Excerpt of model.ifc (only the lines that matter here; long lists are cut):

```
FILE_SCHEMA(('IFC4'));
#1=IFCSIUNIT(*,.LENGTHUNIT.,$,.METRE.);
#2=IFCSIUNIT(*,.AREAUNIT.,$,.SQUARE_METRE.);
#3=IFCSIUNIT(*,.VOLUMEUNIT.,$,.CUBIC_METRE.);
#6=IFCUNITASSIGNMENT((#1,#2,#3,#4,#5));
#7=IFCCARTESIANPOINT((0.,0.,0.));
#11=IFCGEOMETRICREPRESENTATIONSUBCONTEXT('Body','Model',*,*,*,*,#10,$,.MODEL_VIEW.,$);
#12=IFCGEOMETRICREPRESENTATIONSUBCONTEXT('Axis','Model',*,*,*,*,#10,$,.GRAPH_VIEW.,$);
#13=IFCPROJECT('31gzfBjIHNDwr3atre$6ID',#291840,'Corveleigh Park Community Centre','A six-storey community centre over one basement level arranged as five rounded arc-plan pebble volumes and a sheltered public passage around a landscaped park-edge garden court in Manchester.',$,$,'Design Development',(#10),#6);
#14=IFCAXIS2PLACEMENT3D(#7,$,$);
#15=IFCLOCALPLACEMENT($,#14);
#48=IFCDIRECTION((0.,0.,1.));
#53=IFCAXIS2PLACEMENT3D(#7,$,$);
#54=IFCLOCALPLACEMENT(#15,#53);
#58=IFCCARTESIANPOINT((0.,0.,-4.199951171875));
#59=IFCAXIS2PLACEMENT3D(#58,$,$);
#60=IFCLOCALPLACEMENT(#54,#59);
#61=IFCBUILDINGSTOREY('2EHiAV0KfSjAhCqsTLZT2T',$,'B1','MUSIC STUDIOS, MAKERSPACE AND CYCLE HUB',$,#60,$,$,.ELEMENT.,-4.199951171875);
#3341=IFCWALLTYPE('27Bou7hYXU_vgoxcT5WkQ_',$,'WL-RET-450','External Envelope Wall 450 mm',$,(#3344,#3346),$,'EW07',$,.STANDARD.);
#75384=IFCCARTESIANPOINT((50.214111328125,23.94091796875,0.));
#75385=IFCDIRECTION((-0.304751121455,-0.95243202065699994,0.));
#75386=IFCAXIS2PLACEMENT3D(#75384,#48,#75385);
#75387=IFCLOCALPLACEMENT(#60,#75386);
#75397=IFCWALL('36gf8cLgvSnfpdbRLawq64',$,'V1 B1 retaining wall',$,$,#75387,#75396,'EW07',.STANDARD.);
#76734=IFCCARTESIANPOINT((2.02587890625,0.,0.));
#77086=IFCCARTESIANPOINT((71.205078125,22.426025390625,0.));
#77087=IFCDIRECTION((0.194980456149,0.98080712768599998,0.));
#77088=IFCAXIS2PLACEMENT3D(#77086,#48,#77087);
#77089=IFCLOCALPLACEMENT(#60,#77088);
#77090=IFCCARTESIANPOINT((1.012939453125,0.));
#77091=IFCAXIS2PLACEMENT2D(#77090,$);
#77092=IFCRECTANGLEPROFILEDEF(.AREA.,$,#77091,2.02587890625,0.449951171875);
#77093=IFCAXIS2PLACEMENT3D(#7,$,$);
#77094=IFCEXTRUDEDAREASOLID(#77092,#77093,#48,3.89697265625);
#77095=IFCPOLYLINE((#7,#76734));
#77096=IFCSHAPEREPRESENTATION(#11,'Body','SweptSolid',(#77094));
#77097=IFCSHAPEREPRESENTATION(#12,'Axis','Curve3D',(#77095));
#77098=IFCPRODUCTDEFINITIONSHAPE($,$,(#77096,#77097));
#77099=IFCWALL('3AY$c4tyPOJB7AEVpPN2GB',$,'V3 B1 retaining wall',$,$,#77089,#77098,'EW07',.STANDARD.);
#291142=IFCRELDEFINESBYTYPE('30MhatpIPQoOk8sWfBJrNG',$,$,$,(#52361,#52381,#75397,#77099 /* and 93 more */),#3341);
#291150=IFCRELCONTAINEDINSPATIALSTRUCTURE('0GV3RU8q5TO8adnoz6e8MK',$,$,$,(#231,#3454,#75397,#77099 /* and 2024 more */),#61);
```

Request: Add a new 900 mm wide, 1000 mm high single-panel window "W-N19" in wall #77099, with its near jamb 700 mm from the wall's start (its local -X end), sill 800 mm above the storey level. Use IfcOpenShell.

```python
import numpy as np
import ifcopenshell
import ifcopenshell.api.feature
import ifcopenshell.api.geometry
import ifcopenshell.api.root
import ifcopenshell.api.spatial
import ifcopenshell.geom
import ifcopenshell.util.element
import ifcopenshell.util.placement
import ifcopenshell.util.representation
import ifcopenshell.util.shape
import ifcopenshell.util.unit

model = ifcopenshell.open("model.ifc")
unit_scale = ifcopenshell.util.unit.calculate_unit_scale(model)
settings = ifcopenshell.geom.settings()


def volume(element):
    """Net volume in cubic metres, openings subtracted."""
    shape = ifcopenshell.geom.create_shape(settings, element)
    return ifcopenshell.util.shape.get_volume(shape.geometry)


wall = model.by_guid("3AY$c4tyPOJB7AEVpPN2GB")
storey = ifcopenshell.util.element.get_container(wall, ifc_class="IfcBuildingStorey")
context = ifcopenshell.util.representation.get_context(model, "Model", "Body", "MODEL_VIEW")
before = volume(wall)

width, height, from_end, sill = 0.9, 1, 0.7, 0.8  # metres

# The wall runs along its own X axis, and the end named is its -X end.
wall_shape = ifcopenshell.geom.create_shape(settings, wall)
x, y, z = ifcopenshell.util.shape.get_vertices(wall_shape.geometry).T
start = x.min() + from_end
face, thickness = float(y.min()), float(y.max() - y.min())
wall_matrix = ifcopenshell.util.placement.get_local_placement(wall.ObjectPlacement)
level = ifcopenshell.util.placement.get_local_placement(storey.ObjectPlacement)[2, 3]


def in_wall(x, y):
    """Placement at x, y metres in the wall's axes, at sill height."""
    matrix = wall_matrix.copy()
    matrix[:, 3] = wall_matrix @ np.array([x / unit_scale, y / unit_scale, 0.0, 1.0])
    matrix[2, 3] = level + sill / unit_scale
    return matrix


# Opening: a box that overshoots both wall faces by 50 mm.
opening = ifcopenshell.api.root.create_entity(model, ifc_class="IfcOpeningElement", predefined_type="OPENING")
box = ifcopenshell.api.geometry.add_wall_representation(
    model, context=context, length=width, height=height, thickness=thickness + 0.1
)
ifcopenshell.api.geometry.assign_representation(model, product=opening, representation=box)
ifcopenshell.api.geometry.edit_object_placement(model, product=opening, matrix=in_wall(start, face - 0.05), is_si=False)
ifcopenshell.api.feature.add_feature(model, feature=opening, element=wall)

window = ifcopenshell.api.root.create_entity(model, ifc_class="IfcWindow", name="W-N19", predefined_type="WINDOW")
window.OverallWidth, window.OverallHeight = width / unit_scale, height / unit_scale
window.PartitioningType = "SINGLE_PANEL"
body = ifcopenshell.api.geometry.add_window_representation(
    model,
    context=context,
    overall_width=window.OverallWidth,
    overall_height=window.OverallHeight,
    partition_type="SINGLE_PANEL",
)
ifcopenshell.api.geometry.assign_representation(model, product=window, representation=body)
ifcopenshell.api.spatial.assign_container(model, products=[window], relating_structure=storey)
ifcopenshell.api.feature.add_filling(model, opening=opening, element=window)

# Centre the window in the wall's thickness.
ifcopenshell.api.geometry.edit_object_placement(model, product=window, matrix=in_wall(start, face), is_si=False)
window_shape = ifcopenshell.geom.create_shape(settings, window)
depth = ifcopenshell.util.shape.get_vertices(window_shape.geometry)[:, 1]
offset = face + thickness / 2 - (depth.min() + depth.max()) / 2
ifcopenshell.api.geometry.edit_object_placement(model, product=window, matrix=in_wall(start, offset), is_si=False)

after = volume(wall)

print(f"wall volume {before:.3f} -> {after:.3f} m3")

model.write("model_v2.ifc")
```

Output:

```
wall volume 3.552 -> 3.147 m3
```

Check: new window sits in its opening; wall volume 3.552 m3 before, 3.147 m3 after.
